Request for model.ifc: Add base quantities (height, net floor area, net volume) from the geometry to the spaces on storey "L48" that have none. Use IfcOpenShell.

First a look at what the model holds.

```python
import ifcopenshell
import ifcopenshell.util.element
import ifcopenshell.util.unit

model = ifcopenshell.open("model.ifc")
print(model.schema)
for unit_type in ("LENGTHUNIT", "AREAUNIT", "VOLUMEUNIT"):
    print(unit_type, ifcopenshell.util.unit.calculate_unit_scale(model, unit_type))
storey = next(s for s in model.by_type("IfcBuildingStorey") if s.Name == "L48")
spaces = [e for e in ifcopenshell.util.element.get_decomposition(storey) if e.is_a("IfcSpace")]
for e in sorted(spaces, key=lambda e: e.id()):
    print(e.id(), e.is_a(), e.Name, list(ifcopenshell.util.element.get_psets(e, qtos_only=True)), sep=" | ")
```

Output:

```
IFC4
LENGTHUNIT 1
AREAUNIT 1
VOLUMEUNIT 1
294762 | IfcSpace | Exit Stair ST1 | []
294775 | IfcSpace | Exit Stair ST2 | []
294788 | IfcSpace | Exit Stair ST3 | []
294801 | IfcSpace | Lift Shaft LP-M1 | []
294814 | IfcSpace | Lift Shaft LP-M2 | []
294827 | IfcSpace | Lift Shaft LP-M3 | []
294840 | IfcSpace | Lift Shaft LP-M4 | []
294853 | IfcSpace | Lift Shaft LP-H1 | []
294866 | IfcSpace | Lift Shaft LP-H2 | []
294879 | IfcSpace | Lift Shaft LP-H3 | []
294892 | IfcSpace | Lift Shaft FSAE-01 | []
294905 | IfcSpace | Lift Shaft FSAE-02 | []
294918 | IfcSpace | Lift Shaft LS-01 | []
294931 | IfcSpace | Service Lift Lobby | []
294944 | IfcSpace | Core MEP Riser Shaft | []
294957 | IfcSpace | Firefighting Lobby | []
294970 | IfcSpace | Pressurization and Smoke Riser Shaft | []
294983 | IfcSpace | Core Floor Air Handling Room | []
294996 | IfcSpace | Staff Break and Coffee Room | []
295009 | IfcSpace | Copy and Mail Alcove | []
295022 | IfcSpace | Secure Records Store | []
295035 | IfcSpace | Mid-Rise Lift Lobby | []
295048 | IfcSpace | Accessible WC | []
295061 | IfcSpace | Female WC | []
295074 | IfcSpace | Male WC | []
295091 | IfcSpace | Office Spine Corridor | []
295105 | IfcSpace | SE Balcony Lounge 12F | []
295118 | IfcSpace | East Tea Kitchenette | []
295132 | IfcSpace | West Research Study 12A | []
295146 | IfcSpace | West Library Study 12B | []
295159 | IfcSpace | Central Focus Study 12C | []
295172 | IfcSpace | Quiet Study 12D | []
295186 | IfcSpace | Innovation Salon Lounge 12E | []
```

```python
import ifcopenshell
import ifcopenshell.api.pset
import ifcopenshell.geom
import ifcopenshell.util.element
import ifcopenshell.util.shape
import ifcopenshell.util.unit

model = ifcopenshell.open("model.ifc")
unit_scale = ifcopenshell.util.unit.calculate_unit_scale(model)
area_scale = ifcopenshell.util.unit.calculate_unit_scale(model, "AREAUNIT")
volume_scale = ifcopenshell.util.unit.calculate_unit_scale(model, "VOLUMEUNIT")
settings = ifcopenshell.geom.settings()

storey = next(s for s in model.by_type("IfcBuildingStorey") if s.Name == "L48")
spaces = [e for e in ifcopenshell.util.element.get_decomposition(storey) if e.is_a("IfcSpace")]

for e in sorted(spaces, key=lambda e: e.id()):
    if ifcopenshell.util.element.get_psets(e, qtos_only=True, should_inherit=False):
        continue
    # Geometry comes back in metres, in the element's own axes.
    shape = ifcopenshell.geom.create_shape(settings, e)
    values = {
        "Height": ifcopenshell.util.shape.get_z(shape.geometry) / unit_scale,
        "NetFloorArea": ifcopenshell.util.shape.get_footprint_area(shape.geometry) / area_scale,
        "NetVolume": ifcopenshell.util.shape.get_volume(shape.geometry) / volume_scale,
    }
    qto = ifcopenshell.api.pset.add_qto(model, product=e, name="Qto_SpaceBaseQuantities")
    ifcopenshell.api.pset.edit_qto(model, qto=qto, properties=values)
    print(e.id(), {k: round(v, 3) for k, v in values.items()})

model.write("model_updated.ifc")
```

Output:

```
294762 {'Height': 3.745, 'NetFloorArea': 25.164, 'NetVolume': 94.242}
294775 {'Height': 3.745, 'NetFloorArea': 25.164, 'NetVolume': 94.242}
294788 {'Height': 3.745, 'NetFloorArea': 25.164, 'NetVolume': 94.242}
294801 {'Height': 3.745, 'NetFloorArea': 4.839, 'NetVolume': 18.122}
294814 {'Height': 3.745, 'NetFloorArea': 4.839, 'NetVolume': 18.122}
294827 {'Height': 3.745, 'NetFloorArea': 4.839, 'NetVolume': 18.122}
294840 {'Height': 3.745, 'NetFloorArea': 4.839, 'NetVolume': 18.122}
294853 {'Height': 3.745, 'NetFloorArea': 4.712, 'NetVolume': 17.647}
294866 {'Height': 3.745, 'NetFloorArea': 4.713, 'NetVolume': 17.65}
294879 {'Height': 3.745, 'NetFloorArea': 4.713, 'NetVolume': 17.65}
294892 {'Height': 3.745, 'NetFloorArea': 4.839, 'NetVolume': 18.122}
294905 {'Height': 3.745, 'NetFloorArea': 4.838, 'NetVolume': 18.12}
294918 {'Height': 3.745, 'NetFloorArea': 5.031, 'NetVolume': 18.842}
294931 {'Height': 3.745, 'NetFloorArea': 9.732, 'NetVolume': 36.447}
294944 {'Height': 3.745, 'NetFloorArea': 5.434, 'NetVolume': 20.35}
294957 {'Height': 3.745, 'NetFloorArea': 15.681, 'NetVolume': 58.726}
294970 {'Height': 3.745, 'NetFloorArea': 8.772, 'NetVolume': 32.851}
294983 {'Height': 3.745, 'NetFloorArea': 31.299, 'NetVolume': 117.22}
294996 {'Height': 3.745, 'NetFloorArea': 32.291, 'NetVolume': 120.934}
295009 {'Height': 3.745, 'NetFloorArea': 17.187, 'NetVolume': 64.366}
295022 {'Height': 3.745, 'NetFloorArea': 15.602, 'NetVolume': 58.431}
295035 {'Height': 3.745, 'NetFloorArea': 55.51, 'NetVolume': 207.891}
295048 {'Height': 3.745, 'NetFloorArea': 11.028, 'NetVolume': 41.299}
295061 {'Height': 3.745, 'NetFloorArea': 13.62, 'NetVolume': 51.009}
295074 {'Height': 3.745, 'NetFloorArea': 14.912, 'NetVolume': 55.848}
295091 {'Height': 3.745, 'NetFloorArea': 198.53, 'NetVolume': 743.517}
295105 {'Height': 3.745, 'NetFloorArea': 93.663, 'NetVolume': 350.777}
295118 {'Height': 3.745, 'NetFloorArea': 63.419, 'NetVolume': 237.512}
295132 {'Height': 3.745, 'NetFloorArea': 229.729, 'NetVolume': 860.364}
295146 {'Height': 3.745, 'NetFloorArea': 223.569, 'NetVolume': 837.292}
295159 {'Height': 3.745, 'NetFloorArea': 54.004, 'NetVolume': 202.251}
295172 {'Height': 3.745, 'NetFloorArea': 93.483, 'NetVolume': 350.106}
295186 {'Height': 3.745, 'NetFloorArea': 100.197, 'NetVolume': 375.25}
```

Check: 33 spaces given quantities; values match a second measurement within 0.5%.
